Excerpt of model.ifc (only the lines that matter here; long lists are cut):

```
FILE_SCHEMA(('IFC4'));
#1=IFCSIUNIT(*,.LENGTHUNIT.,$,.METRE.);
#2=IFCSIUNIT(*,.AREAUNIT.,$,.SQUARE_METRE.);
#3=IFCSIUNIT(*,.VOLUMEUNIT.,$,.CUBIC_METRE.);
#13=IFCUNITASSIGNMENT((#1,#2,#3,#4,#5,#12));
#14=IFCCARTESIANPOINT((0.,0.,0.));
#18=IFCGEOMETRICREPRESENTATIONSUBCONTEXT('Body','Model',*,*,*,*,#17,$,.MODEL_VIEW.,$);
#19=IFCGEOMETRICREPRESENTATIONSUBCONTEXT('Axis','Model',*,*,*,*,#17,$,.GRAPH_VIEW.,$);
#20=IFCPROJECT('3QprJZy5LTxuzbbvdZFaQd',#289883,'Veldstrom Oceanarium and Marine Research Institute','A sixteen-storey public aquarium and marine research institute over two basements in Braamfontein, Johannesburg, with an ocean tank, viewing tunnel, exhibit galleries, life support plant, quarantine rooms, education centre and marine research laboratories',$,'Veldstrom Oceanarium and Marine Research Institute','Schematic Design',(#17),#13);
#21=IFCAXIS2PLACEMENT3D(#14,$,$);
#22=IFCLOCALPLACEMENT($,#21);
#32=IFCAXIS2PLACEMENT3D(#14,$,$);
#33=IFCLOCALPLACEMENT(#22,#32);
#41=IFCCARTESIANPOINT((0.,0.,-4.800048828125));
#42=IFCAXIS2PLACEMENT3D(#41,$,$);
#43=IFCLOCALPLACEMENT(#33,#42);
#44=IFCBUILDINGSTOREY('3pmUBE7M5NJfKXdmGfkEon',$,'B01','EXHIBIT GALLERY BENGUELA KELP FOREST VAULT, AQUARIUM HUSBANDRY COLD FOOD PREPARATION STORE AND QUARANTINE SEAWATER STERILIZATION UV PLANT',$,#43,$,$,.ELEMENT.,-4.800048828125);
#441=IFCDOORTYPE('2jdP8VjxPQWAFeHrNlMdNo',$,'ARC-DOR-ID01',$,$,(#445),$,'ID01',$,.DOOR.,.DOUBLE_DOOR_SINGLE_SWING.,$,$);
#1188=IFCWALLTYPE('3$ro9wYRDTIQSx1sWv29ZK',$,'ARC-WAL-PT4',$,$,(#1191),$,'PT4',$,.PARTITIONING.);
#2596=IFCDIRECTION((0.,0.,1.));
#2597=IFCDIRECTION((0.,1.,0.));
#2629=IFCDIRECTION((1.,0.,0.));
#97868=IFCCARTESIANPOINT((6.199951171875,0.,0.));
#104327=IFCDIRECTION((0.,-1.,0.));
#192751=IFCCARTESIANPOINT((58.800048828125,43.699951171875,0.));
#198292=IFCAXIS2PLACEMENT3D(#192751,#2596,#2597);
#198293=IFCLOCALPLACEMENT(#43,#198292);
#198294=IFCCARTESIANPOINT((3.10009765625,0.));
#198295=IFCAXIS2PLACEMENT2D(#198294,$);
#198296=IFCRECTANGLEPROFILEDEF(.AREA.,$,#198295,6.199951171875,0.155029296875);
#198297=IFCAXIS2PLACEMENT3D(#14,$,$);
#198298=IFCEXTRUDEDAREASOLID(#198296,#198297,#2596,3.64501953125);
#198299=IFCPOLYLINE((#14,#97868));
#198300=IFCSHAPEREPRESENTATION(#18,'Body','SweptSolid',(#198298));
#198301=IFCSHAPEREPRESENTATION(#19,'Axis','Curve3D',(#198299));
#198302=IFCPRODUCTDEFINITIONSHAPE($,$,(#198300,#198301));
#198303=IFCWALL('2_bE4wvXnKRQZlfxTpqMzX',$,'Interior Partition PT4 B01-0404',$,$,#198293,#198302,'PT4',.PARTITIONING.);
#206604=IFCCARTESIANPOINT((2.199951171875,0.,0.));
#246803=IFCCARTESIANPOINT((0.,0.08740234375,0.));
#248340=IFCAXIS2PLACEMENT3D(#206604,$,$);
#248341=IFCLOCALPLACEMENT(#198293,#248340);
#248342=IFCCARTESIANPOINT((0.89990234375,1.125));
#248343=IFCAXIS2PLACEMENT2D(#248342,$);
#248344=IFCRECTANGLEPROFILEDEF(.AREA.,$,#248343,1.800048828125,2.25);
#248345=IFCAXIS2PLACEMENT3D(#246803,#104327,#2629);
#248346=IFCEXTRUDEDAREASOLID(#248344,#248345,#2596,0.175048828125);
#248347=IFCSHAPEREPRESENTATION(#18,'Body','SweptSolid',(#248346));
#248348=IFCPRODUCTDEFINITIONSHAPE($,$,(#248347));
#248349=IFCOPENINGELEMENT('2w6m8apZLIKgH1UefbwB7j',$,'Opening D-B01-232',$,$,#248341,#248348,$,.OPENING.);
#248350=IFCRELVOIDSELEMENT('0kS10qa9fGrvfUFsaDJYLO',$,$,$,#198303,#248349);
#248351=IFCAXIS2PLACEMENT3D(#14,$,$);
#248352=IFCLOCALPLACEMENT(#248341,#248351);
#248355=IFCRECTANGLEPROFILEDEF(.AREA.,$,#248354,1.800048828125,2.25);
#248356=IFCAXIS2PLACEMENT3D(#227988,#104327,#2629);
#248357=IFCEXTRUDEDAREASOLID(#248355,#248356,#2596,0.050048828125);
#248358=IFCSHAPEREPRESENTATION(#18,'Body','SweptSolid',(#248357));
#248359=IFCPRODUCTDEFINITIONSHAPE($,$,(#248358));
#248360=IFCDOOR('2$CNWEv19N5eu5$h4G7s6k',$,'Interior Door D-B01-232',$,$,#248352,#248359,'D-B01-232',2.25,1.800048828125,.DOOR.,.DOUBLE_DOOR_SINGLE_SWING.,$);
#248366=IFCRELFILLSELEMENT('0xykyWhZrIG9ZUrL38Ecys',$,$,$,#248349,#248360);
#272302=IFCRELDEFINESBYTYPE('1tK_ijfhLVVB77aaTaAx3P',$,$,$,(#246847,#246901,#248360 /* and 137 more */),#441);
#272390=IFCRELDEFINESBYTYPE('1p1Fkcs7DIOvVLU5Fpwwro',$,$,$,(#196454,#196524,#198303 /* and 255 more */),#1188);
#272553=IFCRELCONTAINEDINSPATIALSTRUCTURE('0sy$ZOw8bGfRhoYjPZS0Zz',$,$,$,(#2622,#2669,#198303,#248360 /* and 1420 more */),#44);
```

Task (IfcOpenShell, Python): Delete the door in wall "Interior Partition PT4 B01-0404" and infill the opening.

```python
import ifcopenshell
import ifcopenshell.api.feature
import ifcopenshell.api.root
import ifcopenshell.geom
import ifcopenshell.util.shape

model = ifcopenshell.open("model.ifc")
settings = ifcopenshell.geom.settings()


def volume(element):
    """Net volume in cubic metres, openings subtracted."""
    shape = ifcopenshell.geom.create_shape(settings, element)
    return ifcopenshell.util.shape.get_volume(shape.geometry)


door = model.by_guid("2$CNWEv19N5eu5$h4G7s6k")
opening = door.FillsVoids[0].RelatingOpeningElement
wall = opening.VoidsElements[0].RelatingBuildingElement
before = volume(wall)

ifcopenshell.api.root.remove_product(model, product=door)
ifcopenshell.api.feature.remove_feature(model, feature=opening)

after = volume(wall)

print(f"wall volume {before:.3f} -> {after:.3f} m3")

model.write("model_edited.ifc")
```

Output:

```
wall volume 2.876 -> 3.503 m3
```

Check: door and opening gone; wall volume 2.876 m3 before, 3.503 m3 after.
